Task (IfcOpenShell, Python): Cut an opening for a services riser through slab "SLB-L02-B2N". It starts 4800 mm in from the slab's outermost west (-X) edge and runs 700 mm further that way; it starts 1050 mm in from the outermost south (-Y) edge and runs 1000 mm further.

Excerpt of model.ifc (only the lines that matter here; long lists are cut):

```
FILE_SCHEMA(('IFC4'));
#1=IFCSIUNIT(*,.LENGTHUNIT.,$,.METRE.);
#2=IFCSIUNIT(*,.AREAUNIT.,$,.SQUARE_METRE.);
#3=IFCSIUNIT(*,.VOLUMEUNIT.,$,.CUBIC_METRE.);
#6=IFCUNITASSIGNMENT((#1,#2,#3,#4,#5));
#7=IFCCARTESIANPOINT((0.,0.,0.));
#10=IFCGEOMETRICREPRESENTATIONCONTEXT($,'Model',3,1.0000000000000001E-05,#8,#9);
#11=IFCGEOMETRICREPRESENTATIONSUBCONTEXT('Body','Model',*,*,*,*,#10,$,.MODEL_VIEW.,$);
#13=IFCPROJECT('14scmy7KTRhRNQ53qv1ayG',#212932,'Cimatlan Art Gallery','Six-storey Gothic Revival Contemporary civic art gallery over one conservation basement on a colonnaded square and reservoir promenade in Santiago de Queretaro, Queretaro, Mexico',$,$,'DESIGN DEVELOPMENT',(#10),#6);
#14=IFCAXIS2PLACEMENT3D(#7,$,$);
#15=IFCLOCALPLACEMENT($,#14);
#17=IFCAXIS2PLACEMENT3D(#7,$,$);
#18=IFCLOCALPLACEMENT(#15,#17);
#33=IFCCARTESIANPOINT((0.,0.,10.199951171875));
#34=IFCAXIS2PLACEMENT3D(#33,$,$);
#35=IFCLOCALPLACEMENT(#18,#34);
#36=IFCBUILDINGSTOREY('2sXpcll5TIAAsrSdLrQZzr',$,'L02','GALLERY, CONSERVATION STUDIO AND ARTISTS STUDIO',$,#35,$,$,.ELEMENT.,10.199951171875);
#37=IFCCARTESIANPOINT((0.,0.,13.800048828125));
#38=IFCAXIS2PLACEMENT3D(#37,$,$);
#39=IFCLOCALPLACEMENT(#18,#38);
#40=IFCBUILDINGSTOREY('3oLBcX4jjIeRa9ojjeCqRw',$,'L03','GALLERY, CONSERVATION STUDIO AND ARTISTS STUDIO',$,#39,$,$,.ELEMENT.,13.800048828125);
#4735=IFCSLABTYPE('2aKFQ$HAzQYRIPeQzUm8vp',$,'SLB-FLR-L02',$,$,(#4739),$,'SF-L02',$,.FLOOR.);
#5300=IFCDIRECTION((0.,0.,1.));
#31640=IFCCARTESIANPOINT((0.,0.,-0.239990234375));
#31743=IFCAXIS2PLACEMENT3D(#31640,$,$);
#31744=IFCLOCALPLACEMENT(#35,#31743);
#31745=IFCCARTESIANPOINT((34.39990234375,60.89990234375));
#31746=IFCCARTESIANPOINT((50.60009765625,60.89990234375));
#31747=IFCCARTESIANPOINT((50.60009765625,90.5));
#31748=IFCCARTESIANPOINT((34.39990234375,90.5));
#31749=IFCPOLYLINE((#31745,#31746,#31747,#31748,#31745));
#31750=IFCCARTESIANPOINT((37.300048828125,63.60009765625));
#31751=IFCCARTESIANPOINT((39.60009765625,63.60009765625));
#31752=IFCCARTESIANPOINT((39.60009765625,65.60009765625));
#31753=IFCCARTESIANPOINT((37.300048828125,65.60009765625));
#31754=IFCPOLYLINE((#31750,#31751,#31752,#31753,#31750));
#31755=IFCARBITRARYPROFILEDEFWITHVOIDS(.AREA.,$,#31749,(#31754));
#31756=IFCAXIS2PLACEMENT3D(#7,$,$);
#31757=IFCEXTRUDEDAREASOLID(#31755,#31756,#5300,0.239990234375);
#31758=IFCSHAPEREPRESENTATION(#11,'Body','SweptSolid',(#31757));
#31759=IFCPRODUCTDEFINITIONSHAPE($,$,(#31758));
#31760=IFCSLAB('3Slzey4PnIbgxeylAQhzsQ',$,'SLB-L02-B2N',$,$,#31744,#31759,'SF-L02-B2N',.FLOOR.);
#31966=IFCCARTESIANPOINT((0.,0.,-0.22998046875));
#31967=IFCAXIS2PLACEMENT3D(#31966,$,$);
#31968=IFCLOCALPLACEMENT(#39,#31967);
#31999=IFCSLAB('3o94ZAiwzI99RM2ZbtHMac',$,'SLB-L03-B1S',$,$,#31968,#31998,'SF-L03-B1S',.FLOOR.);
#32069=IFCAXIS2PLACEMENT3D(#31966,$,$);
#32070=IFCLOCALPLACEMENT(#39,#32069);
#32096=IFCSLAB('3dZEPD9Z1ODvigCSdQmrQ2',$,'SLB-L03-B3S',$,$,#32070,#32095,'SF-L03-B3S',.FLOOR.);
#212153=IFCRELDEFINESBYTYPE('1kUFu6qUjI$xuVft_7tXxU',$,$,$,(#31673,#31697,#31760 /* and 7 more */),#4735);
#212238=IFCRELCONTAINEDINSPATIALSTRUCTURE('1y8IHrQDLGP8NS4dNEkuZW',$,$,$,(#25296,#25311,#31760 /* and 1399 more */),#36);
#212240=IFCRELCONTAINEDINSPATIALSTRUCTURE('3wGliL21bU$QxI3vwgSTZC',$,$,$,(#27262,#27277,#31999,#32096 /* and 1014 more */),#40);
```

```python
import numpy as np
import ifcopenshell
import ifcopenshell.api.feature
import ifcopenshell.api.geometry
import ifcopenshell.api.root
import ifcopenshell.geom
import ifcopenshell.util.placement
import ifcopenshell.util.representation
import ifcopenshell.util.shape
import ifcopenshell.util.unit

model = ifcopenshell.open("model.ifc")
unit_scale = ifcopenshell.util.unit.calculate_unit_scale(model)
settings = ifcopenshell.geom.settings()


def volume(element):
    """Net volume in cubic metres, openings subtracted."""
    shape = ifcopenshell.geom.create_shape(settings, element)
    return ifcopenshell.util.shape.get_volume(shape.geometry)


slab = model.by_guid("3Slzey4PnIbgxeylAQhzsQ")
before = volume(slab)

# Extent in the slab's own axes, in metres. The edges named are its -X and -Y sides.
slab_shape = ifcopenshell.geom.create_shape(settings, slab)
vertices = ifcopenshell.util.shape.get_vertices(slab_shape.geometry)
x_min, y_min, bottom = vertices.min(axis=0)
top = vertices[:, 2].max()

opening = ifcopenshell.api.root.create_entity(model, ifc_class="IfcOpeningElement", name="Services riser opening", predefined_type="OPENING")
context = ifcopenshell.util.representation.get_context(model, "Model", "Body", "MODEL_VIEW")
width, depth = 0.7, 1
outline = [(0.0, 0.0), (width, 0.0), (width, depth), (0.0, depth), (0.0, 0.0)]
# Overshoot both faces by 50 mm so the cut is clean.
shape = ifcopenshell.api.geometry.add_slab_representation(
    model, context=context, depth=top - bottom + 0.1, polyline=outline
)
ifcopenshell.api.geometry.assign_representation(model, product=opening, representation=shape)

matrix = ifcopenshell.util.placement.get_local_placement(slab.ObjectPlacement)
matrix[:, 3] = matrix @ np.append(np.array([x_min + 4.8, y_min + 1.05, bottom - 0.05]) / unit_scale, 1.0)
ifcopenshell.api.geometry.edit_object_placement(model, product=opening, matrix=matrix, is_si=False)
ifcopenshell.api.feature.add_feature(model, feature=opening, element=slab)

after = volume(slab)

print(f"slab volume {before:.3f} -> {after:.3f} m3")

model.write("model_v2.ifc")
```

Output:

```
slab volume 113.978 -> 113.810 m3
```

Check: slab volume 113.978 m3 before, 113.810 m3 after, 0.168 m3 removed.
